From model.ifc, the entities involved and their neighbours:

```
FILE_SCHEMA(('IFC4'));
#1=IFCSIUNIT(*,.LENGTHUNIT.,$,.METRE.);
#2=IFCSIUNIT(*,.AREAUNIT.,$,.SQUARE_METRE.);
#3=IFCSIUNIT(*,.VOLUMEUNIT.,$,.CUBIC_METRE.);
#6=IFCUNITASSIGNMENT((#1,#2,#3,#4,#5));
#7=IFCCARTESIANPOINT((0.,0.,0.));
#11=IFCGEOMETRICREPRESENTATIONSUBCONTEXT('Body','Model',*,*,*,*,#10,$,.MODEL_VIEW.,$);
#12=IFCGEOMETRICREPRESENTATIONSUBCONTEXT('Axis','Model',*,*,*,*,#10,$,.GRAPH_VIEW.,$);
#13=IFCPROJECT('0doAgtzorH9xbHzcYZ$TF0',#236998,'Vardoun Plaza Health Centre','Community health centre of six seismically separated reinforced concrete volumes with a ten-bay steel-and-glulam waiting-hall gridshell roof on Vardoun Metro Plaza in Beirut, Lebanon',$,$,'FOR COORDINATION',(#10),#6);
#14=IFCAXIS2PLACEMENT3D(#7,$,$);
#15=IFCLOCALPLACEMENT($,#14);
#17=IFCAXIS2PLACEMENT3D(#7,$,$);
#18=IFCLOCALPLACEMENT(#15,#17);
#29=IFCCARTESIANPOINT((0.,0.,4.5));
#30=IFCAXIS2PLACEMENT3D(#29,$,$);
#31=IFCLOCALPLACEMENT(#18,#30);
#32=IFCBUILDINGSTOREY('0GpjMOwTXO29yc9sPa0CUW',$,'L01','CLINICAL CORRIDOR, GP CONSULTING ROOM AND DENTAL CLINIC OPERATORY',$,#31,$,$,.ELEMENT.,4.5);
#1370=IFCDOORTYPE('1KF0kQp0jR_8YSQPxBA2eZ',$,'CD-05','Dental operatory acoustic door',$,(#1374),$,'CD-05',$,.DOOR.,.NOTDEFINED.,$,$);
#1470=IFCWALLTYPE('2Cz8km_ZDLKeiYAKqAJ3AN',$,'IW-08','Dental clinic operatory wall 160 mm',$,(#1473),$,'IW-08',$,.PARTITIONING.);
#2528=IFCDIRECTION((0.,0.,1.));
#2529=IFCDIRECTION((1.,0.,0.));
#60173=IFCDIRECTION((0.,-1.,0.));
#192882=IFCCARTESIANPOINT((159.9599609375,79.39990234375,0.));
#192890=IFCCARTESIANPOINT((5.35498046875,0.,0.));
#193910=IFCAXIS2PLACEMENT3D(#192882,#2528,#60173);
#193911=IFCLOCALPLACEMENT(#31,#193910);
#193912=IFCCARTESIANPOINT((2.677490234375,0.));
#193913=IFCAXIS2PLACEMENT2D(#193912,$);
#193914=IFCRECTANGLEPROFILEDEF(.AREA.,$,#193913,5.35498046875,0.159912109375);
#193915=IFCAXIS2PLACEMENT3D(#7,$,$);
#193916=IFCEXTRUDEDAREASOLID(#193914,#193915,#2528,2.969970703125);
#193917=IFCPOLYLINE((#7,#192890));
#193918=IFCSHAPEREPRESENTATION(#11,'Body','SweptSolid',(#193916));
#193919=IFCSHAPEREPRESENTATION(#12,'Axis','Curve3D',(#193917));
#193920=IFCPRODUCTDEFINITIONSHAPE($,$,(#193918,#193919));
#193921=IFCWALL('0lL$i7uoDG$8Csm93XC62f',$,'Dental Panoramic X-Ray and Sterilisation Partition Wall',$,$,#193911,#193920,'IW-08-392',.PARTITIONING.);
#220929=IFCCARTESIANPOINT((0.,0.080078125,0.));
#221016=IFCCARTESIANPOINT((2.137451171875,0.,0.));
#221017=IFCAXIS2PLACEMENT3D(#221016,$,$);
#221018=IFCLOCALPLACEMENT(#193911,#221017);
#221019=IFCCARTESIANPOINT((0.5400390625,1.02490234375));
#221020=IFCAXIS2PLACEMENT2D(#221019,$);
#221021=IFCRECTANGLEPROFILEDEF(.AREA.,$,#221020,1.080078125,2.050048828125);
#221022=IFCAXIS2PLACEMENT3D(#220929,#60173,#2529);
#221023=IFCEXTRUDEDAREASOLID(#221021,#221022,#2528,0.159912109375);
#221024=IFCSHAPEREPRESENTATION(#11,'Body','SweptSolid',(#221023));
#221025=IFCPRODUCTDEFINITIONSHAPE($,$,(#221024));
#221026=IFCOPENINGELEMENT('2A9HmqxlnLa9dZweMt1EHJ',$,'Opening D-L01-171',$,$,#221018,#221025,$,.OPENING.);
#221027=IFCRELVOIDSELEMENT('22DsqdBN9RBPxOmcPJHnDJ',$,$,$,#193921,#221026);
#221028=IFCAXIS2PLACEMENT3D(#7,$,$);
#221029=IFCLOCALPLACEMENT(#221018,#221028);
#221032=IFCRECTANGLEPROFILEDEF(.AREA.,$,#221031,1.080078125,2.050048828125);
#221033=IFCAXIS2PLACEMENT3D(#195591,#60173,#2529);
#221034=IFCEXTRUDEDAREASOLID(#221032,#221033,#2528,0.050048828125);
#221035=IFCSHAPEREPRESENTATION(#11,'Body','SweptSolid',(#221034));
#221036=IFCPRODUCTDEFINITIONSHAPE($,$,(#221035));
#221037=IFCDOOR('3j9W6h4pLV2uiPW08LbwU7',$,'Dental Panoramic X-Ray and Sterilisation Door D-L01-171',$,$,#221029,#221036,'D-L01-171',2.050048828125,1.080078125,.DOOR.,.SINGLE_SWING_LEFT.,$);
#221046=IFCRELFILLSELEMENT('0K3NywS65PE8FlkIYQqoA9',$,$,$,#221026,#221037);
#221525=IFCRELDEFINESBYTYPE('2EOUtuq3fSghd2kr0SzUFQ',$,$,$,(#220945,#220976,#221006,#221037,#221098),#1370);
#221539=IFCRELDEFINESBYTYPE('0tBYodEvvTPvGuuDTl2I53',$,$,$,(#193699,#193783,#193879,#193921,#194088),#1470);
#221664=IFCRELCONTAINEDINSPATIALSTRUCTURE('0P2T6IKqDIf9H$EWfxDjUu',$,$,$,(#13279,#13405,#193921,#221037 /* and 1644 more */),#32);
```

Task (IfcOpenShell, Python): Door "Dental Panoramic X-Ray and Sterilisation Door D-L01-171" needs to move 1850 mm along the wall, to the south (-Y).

```python
import ifcopenshell
import ifcopenshell.api.geometry
import ifcopenshell.util.placement

model = ifcopenshell.open("model.ifc")

door = model.by_guid("3j9W6h4pLV2uiPW08LbwU7")
opening = door.FillsVoids[0].RelatingOpeningElement
wall = opening.VoidsElements[0].RelatingBuildingElement

wall_matrix = ifcopenshell.util.placement.get_local_placement(wall.ObjectPlacement)
shift = wall_matrix[:3, 0] * 1.85
before = ifcopenshell.util.placement.get_local_placement(door.ObjectPlacement)[:3, 3].copy()

# The door is placed relative to its opening, so it follows when the opening moves.
matrix = ifcopenshell.util.placement.get_local_placement(opening.ObjectPlacement)
matrix[:3, 3] += shift
ifcopenshell.api.geometry.edit_object_placement(
    model, product=opening, matrix=matrix, is_si=False, should_transform_children=True
)

after = ifcopenshell.util.placement.get_local_placement(door.ObjectPlacement)[:3, 3]
print("door moved by", (after - before).round(3) + 0.0)

model.write("model-out.ifc")
```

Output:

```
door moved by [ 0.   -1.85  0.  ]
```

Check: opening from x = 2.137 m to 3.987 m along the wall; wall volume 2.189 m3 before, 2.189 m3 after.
